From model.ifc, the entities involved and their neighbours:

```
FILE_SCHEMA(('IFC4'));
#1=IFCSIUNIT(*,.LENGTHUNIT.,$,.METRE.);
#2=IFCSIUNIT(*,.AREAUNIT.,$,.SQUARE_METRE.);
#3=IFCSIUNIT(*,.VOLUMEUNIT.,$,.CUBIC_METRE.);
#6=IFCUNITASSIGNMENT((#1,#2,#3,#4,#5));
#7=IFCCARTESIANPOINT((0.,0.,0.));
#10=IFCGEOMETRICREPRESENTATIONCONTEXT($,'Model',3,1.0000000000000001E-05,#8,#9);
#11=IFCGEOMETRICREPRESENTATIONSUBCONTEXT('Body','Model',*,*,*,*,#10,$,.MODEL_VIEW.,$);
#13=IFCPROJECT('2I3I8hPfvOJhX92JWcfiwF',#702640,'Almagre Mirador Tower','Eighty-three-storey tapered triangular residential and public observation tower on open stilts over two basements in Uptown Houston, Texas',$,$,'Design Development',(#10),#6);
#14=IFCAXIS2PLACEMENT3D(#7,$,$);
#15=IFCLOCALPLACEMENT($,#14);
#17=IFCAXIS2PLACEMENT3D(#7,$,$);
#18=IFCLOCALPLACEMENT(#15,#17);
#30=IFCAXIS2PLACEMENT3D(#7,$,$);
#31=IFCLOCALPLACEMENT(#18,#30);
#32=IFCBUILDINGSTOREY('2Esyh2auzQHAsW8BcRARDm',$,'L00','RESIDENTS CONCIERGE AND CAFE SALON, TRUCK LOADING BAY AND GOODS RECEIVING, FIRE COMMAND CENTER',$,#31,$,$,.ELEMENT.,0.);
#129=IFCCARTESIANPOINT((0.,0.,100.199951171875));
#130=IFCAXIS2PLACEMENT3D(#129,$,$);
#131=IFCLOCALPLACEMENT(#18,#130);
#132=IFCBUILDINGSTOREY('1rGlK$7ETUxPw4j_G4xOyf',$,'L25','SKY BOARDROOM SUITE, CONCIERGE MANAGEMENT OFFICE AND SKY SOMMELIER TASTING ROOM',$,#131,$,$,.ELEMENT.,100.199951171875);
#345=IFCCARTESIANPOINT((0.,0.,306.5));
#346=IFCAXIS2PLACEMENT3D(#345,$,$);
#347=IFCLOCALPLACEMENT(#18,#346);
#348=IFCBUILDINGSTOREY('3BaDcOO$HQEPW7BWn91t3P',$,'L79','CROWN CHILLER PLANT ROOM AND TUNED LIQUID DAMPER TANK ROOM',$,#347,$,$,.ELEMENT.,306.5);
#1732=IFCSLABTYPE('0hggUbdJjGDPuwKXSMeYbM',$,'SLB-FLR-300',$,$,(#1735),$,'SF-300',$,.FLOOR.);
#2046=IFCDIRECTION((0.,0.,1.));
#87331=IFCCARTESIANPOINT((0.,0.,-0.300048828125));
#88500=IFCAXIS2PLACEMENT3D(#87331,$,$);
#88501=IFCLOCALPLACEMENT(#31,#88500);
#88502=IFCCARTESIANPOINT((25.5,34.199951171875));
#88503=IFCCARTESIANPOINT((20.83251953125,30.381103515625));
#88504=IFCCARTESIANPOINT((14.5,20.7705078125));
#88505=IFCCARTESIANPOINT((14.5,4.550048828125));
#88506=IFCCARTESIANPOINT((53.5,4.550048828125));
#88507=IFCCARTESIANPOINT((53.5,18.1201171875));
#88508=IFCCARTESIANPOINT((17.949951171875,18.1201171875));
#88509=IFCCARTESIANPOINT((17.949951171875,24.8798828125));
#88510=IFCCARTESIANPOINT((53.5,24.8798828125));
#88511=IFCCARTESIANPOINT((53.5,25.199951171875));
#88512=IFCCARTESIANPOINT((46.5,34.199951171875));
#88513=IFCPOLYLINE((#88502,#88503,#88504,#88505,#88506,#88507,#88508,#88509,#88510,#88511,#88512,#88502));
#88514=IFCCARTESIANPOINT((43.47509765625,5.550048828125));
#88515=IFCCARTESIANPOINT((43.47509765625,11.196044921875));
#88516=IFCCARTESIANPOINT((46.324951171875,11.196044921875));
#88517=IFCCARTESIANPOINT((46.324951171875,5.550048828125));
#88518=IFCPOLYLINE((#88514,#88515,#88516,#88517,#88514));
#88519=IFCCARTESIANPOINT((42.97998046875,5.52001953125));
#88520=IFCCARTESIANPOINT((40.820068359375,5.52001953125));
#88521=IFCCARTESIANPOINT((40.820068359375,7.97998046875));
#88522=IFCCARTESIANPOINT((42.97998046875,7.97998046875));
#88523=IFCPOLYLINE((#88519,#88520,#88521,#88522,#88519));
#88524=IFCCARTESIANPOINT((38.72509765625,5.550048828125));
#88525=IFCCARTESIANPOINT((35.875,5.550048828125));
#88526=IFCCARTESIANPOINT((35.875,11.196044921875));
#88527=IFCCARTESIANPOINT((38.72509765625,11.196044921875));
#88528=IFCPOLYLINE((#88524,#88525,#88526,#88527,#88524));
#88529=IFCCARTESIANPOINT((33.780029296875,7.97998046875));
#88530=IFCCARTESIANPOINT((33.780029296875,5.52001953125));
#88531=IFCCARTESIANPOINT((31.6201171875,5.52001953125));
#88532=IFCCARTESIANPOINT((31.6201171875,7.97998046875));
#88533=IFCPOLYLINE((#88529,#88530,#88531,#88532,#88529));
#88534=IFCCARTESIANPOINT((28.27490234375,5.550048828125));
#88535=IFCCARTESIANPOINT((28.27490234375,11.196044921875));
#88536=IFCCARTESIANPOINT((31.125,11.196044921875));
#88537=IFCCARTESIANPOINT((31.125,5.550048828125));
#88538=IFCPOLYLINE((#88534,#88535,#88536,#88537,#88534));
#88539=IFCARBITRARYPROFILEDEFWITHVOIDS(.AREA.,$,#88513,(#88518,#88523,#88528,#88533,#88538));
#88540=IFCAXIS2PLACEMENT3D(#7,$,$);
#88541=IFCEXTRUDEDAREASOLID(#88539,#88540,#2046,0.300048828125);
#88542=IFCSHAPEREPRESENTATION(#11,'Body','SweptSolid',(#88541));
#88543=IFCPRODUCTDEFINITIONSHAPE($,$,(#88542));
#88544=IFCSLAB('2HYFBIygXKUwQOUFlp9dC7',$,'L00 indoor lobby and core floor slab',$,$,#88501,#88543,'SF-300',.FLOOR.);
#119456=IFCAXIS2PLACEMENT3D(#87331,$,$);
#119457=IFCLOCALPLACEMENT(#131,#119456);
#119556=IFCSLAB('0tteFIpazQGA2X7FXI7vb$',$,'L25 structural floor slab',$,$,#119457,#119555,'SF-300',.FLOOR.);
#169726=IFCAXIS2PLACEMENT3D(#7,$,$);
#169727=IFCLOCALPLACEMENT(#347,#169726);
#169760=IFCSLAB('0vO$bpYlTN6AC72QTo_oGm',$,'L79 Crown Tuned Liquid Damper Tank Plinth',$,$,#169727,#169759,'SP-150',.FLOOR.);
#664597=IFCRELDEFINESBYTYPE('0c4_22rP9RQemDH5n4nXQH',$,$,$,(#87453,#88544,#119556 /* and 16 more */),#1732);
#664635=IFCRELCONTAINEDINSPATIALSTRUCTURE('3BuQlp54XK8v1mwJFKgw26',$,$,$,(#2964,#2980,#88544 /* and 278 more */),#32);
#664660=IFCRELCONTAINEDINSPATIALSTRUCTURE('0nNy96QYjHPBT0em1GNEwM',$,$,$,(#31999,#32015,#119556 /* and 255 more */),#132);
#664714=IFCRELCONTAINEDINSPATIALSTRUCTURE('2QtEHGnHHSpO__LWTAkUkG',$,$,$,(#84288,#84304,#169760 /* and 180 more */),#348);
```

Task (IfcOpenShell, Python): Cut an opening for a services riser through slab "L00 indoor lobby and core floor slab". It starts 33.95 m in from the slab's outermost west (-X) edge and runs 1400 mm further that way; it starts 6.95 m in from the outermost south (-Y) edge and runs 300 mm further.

```python
import numpy as np
import ifcopenshell
import ifcopenshell.api.feature
import ifcopenshell.api.geometry
import ifcopenshell.api.root
import ifcopenshell.geom
import ifcopenshell.util.placement
import ifcopenshell.util.representation
import ifcopenshell.util.shape
import ifcopenshell.util.unit

model = ifcopenshell.open("model.ifc")
unit_scale = ifcopenshell.util.unit.calculate_unit_scale(model)
settings = ifcopenshell.geom.settings()


def volume(element):
    """Net volume in cubic metres, openings subtracted."""
    shape = ifcopenshell.geom.create_shape(settings, element)
    return ifcopenshell.util.shape.get_volume(shape.geometry)


slab = model.by_guid("2HYFBIygXKUwQOUFlp9dC7")
before = volume(slab)

# Extent in the slab's own axes, in metres. The edges named are its -X and -Y sides.
slab_shape = ifcopenshell.geom.create_shape(settings, slab)
vertices = ifcopenshell.util.shape.get_vertices(slab_shape.geometry)
x_min, y_min, bottom = vertices.min(axis=0)
top = vertices[:, 2].max()

opening = ifcopenshell.api.root.create_entity(model, ifc_class="IfcOpeningElement", name="Services riser opening", predefined_type="OPENING")
context = ifcopenshell.util.representation.get_context(model, "Model", "Body", "MODEL_VIEW")
width, depth = 1.4, 0.3
outline = [(0.0, 0.0), (width, 0.0), (width, depth), (0.0, depth), (0.0, 0.0)]
# Overshoot both faces by 50 mm so the cut is clean.
shape = ifcopenshell.api.geometry.add_slab_representation(
    model, context=context, depth=top - bottom + 0.1, polyline=outline
)
ifcopenshell.api.geometry.assign_representation(model, product=opening, representation=shape)

matrix = ifcopenshell.util.placement.get_local_placement(slab.ObjectPlacement)
matrix[:, 3] = matrix @ np.append(np.array([x_min + 33.95, y_min + 6.95, bottom - 0.05]) / unit_scale, 1.0)
ifcopenshell.api.geometry.edit_object_placement(model, product=opening, matrix=matrix, is_si=False)
ifcopenshell.api.feature.add_feature(model, feature=opening, element=slab)

after = volume(slab)

print(f"slab volume {before:.3f} -> {after:.3f} m3")

model.write("model_rev.ifc")
```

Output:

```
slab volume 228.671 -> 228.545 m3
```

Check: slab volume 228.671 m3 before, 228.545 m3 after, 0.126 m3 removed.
